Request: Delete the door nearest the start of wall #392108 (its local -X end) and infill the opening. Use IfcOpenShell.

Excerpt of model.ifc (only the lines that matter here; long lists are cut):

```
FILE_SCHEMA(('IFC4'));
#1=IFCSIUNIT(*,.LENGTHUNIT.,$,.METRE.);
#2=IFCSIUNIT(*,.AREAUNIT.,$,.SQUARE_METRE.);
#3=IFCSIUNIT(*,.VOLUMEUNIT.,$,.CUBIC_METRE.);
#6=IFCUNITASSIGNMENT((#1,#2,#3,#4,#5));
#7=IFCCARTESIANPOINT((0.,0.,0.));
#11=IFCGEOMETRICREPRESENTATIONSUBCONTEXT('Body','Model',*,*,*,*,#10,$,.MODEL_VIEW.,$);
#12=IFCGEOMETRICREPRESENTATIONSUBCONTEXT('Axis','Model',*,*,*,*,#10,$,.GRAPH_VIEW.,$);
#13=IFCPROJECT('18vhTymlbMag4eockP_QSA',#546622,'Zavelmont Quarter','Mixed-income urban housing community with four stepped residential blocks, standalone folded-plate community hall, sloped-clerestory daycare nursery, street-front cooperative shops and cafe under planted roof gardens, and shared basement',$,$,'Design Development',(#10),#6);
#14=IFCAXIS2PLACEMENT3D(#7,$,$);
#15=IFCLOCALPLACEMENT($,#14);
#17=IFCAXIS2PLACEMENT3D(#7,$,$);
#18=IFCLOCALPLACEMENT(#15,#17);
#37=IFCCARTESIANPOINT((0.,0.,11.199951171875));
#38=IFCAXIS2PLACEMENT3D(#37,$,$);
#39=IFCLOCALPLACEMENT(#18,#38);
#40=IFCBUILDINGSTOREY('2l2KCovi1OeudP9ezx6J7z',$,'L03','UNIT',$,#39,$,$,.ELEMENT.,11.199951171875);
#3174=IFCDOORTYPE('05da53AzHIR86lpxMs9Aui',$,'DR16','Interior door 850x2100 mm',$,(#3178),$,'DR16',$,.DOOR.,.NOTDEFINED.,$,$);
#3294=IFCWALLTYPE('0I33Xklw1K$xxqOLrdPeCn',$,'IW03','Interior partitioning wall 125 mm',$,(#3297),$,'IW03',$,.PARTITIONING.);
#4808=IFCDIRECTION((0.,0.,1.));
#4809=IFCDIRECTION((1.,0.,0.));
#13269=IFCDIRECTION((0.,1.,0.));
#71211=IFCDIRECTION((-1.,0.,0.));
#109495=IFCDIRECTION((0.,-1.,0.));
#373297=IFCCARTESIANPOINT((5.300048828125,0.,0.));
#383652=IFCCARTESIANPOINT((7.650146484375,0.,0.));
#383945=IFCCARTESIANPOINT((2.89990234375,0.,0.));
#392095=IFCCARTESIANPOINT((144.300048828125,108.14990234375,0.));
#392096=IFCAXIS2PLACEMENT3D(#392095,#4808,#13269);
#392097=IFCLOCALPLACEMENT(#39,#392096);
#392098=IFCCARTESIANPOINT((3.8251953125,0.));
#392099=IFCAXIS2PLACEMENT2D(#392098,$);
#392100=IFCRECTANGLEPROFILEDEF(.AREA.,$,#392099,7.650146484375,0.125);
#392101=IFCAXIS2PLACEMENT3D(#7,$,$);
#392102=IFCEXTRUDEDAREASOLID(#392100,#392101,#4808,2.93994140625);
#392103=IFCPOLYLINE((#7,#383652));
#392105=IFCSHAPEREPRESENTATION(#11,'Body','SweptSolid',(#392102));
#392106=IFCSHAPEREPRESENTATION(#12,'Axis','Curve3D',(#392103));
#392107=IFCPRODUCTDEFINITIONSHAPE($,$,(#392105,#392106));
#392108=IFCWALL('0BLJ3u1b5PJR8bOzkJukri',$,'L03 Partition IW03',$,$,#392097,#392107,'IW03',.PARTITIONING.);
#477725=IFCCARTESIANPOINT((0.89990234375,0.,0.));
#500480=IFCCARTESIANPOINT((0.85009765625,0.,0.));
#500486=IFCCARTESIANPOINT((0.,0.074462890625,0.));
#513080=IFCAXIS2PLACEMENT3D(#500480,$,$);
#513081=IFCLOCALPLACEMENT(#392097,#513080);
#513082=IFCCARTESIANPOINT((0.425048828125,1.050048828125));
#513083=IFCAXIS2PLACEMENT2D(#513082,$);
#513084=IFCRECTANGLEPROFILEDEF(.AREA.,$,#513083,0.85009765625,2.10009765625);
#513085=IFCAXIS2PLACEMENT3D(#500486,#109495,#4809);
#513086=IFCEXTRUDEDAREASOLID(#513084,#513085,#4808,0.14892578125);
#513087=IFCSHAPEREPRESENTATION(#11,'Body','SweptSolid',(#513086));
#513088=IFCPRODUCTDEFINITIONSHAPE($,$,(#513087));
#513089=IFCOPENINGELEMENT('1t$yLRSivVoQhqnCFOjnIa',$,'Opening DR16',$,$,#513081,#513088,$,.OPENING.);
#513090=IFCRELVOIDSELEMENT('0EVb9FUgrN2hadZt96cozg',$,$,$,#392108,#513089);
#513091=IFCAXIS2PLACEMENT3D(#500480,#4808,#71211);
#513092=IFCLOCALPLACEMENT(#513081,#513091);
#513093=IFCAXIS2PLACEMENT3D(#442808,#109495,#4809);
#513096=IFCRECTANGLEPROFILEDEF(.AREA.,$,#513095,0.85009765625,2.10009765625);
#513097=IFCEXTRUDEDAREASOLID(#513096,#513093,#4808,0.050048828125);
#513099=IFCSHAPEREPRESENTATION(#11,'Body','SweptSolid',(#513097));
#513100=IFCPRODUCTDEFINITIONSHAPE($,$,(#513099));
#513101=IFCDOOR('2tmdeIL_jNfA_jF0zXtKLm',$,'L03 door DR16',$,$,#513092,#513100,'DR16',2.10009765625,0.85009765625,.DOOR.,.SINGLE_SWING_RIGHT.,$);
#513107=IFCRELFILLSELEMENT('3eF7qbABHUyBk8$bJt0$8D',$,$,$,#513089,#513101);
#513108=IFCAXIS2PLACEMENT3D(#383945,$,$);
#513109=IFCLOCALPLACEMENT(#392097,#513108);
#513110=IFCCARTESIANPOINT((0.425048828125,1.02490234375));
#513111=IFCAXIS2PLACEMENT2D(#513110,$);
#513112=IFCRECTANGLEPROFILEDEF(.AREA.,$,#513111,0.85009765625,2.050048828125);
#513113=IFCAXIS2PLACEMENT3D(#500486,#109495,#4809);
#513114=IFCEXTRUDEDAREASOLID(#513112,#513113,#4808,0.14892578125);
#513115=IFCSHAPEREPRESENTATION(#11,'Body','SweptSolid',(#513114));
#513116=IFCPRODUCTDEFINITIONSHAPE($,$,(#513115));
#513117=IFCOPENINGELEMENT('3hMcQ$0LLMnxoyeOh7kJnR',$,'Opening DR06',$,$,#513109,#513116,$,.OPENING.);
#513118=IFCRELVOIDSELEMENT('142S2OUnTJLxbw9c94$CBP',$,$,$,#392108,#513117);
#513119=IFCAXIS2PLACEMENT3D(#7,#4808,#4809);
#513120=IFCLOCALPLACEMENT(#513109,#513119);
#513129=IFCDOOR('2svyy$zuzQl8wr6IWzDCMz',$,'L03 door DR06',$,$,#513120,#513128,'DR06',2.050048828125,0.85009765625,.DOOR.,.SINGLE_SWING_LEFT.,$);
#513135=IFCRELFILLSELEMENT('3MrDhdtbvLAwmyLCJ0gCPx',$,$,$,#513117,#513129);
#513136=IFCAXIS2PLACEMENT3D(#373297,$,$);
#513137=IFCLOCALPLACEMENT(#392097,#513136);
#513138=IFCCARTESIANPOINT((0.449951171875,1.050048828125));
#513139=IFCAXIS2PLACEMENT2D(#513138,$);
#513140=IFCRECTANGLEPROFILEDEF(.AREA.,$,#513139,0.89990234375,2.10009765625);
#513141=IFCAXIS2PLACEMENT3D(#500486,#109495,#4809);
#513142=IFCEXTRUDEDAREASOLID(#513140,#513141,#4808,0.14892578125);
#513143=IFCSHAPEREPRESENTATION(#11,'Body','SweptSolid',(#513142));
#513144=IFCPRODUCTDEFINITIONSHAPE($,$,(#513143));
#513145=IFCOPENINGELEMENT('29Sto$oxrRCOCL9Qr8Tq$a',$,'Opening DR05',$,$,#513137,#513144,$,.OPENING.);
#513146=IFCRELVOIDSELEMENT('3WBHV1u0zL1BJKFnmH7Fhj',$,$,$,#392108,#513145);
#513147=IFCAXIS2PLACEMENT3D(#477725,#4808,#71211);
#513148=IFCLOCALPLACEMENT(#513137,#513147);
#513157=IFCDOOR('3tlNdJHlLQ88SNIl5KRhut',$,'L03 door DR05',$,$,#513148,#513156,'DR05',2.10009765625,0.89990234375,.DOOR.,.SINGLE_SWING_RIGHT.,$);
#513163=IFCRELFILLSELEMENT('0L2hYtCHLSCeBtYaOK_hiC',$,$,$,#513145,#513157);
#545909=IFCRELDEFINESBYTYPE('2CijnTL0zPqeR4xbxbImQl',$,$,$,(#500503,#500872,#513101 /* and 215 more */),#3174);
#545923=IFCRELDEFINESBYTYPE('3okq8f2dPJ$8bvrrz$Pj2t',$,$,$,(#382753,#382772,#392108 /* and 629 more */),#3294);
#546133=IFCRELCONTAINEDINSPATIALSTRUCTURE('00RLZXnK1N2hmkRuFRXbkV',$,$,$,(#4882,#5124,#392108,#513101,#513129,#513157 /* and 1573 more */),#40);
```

```python
import ifcopenshell
import ifcopenshell.api.feature
import ifcopenshell.api.root
import ifcopenshell.geom
import ifcopenshell.util.shape

model = ifcopenshell.open("model.ifc")
settings = ifcopenshell.geom.settings()


def volume(element):
    """Net volume in cubic metres, openings subtracted."""
    shape = ifcopenshell.geom.create_shape(settings, element)
    return ifcopenshell.util.shape.get_volume(shape.geometry)


door = model.by_id(513101)
opening = door.FillsVoids[0].RelatingOpeningElement
wall = opening.VoidsElements[0].RelatingBuildingElement
before = volume(wall)

ifcopenshell.api.root.remove_product(model, product=door)
ifcopenshell.api.feature.remove_feature(model, feature=opening)

after = volume(wall)

print(f"wall volume {before:.3f} -> {after:.3f} m3")

model.write("model_v2.ifc")
```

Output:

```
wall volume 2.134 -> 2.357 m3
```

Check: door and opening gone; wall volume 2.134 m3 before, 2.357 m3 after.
